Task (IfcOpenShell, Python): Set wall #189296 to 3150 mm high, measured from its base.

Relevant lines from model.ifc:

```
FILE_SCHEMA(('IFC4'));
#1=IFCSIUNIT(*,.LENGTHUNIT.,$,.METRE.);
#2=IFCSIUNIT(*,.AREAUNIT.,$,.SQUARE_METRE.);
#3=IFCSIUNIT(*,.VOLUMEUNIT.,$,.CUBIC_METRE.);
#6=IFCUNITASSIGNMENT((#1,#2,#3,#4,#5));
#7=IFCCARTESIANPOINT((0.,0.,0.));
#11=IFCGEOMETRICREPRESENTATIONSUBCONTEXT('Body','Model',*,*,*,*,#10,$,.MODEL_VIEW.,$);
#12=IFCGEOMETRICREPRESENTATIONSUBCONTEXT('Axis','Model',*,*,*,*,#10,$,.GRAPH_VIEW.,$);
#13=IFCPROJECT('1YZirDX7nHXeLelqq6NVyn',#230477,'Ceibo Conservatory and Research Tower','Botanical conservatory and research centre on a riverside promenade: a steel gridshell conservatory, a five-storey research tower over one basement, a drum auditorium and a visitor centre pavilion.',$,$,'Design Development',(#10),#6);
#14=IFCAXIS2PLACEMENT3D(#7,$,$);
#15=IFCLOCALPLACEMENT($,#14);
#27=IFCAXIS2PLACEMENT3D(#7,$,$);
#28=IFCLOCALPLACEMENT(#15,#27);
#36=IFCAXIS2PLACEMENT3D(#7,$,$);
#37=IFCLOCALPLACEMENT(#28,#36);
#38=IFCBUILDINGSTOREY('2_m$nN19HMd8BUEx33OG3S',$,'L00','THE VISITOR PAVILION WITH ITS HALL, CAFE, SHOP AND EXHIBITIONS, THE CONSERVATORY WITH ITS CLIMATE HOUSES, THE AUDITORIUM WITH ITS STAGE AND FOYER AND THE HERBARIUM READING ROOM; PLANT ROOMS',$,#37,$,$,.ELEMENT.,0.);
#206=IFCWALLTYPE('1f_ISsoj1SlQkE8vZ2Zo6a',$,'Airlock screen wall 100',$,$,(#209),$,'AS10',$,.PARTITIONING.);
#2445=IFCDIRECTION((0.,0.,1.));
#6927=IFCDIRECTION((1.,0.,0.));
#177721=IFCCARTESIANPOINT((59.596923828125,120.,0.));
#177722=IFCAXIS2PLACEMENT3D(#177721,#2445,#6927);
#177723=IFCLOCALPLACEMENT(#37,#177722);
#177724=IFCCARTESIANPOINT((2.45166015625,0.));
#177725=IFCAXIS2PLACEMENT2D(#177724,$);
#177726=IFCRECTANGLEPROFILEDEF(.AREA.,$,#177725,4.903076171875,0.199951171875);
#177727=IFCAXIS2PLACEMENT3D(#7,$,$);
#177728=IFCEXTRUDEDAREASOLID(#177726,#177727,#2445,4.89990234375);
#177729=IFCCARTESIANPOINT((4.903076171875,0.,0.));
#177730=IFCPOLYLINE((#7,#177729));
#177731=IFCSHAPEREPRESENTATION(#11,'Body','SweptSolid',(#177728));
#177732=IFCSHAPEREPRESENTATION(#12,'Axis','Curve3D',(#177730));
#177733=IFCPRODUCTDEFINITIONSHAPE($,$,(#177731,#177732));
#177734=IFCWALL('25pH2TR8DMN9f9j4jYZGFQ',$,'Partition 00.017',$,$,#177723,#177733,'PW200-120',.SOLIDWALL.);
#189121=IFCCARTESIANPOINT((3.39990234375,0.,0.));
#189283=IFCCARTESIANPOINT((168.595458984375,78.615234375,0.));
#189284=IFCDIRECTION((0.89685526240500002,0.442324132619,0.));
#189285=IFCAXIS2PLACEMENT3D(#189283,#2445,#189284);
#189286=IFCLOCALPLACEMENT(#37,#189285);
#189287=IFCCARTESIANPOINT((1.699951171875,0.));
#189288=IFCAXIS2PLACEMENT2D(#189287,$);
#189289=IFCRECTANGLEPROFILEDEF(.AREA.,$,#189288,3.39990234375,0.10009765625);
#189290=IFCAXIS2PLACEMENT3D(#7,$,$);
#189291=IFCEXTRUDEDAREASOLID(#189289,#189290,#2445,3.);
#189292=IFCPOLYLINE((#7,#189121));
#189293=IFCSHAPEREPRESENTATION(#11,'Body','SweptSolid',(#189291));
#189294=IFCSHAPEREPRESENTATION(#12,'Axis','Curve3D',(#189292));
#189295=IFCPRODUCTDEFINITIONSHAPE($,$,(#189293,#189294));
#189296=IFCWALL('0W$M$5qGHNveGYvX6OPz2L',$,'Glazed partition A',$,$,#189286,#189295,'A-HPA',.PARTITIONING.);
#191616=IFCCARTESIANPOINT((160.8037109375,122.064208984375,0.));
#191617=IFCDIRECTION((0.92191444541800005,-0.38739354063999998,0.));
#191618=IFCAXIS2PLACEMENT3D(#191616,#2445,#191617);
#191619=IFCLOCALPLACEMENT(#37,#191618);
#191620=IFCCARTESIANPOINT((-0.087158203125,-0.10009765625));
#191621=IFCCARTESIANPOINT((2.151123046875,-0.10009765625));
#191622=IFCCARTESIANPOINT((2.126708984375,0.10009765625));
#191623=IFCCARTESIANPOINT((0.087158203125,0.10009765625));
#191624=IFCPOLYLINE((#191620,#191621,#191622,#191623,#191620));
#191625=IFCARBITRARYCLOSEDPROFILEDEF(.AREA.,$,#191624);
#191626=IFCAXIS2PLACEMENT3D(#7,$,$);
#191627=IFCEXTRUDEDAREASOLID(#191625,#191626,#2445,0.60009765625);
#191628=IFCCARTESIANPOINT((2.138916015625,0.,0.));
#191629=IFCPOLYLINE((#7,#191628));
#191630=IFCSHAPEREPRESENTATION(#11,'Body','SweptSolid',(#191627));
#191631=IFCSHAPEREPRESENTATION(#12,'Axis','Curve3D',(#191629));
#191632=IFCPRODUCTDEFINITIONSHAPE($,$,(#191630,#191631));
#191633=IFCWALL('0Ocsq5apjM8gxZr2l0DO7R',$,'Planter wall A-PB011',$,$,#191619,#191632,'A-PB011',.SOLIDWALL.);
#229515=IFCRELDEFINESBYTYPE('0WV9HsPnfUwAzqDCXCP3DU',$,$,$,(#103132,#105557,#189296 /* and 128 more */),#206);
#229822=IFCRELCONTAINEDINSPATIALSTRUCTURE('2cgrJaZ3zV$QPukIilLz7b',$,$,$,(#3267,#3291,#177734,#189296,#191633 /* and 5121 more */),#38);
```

```python
import ifcopenshell
import ifcopenshell.geom
import ifcopenshell.util.representation
import ifcopenshell.util.shape
import ifcopenshell.util.unit

model = ifcopenshell.open("model.ifc")
unit_scale = ifcopenshell.util.unit.calculate_unit_scale(model)
settings = ifcopenshell.geom.settings()


def volume(element):
    """Net volume in cubic metres, openings subtracted."""
    shape = ifcopenshell.geom.create_shape(settings, element)
    return ifcopenshell.util.shape.get_volume(shape.geometry)


wall = model.by_guid("0W$M$5qGHNveGYvX6OPz2L")
before = volume(wall)

body = ifcopenshell.util.representation.get_representation(wall, "Model", "Body")
solid = body.Items[0]
old_height = solid.Depth
solid.Depth = 3.15 / unit_scale
after = volume(wall)

print(f"height {old_height:g} -> {solid.Depth:g}, volume {before:.3f} -> {after:.3f} m3")

model.write("model_rev.ifc")
```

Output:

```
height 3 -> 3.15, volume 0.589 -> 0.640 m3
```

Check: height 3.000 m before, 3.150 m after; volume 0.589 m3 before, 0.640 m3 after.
